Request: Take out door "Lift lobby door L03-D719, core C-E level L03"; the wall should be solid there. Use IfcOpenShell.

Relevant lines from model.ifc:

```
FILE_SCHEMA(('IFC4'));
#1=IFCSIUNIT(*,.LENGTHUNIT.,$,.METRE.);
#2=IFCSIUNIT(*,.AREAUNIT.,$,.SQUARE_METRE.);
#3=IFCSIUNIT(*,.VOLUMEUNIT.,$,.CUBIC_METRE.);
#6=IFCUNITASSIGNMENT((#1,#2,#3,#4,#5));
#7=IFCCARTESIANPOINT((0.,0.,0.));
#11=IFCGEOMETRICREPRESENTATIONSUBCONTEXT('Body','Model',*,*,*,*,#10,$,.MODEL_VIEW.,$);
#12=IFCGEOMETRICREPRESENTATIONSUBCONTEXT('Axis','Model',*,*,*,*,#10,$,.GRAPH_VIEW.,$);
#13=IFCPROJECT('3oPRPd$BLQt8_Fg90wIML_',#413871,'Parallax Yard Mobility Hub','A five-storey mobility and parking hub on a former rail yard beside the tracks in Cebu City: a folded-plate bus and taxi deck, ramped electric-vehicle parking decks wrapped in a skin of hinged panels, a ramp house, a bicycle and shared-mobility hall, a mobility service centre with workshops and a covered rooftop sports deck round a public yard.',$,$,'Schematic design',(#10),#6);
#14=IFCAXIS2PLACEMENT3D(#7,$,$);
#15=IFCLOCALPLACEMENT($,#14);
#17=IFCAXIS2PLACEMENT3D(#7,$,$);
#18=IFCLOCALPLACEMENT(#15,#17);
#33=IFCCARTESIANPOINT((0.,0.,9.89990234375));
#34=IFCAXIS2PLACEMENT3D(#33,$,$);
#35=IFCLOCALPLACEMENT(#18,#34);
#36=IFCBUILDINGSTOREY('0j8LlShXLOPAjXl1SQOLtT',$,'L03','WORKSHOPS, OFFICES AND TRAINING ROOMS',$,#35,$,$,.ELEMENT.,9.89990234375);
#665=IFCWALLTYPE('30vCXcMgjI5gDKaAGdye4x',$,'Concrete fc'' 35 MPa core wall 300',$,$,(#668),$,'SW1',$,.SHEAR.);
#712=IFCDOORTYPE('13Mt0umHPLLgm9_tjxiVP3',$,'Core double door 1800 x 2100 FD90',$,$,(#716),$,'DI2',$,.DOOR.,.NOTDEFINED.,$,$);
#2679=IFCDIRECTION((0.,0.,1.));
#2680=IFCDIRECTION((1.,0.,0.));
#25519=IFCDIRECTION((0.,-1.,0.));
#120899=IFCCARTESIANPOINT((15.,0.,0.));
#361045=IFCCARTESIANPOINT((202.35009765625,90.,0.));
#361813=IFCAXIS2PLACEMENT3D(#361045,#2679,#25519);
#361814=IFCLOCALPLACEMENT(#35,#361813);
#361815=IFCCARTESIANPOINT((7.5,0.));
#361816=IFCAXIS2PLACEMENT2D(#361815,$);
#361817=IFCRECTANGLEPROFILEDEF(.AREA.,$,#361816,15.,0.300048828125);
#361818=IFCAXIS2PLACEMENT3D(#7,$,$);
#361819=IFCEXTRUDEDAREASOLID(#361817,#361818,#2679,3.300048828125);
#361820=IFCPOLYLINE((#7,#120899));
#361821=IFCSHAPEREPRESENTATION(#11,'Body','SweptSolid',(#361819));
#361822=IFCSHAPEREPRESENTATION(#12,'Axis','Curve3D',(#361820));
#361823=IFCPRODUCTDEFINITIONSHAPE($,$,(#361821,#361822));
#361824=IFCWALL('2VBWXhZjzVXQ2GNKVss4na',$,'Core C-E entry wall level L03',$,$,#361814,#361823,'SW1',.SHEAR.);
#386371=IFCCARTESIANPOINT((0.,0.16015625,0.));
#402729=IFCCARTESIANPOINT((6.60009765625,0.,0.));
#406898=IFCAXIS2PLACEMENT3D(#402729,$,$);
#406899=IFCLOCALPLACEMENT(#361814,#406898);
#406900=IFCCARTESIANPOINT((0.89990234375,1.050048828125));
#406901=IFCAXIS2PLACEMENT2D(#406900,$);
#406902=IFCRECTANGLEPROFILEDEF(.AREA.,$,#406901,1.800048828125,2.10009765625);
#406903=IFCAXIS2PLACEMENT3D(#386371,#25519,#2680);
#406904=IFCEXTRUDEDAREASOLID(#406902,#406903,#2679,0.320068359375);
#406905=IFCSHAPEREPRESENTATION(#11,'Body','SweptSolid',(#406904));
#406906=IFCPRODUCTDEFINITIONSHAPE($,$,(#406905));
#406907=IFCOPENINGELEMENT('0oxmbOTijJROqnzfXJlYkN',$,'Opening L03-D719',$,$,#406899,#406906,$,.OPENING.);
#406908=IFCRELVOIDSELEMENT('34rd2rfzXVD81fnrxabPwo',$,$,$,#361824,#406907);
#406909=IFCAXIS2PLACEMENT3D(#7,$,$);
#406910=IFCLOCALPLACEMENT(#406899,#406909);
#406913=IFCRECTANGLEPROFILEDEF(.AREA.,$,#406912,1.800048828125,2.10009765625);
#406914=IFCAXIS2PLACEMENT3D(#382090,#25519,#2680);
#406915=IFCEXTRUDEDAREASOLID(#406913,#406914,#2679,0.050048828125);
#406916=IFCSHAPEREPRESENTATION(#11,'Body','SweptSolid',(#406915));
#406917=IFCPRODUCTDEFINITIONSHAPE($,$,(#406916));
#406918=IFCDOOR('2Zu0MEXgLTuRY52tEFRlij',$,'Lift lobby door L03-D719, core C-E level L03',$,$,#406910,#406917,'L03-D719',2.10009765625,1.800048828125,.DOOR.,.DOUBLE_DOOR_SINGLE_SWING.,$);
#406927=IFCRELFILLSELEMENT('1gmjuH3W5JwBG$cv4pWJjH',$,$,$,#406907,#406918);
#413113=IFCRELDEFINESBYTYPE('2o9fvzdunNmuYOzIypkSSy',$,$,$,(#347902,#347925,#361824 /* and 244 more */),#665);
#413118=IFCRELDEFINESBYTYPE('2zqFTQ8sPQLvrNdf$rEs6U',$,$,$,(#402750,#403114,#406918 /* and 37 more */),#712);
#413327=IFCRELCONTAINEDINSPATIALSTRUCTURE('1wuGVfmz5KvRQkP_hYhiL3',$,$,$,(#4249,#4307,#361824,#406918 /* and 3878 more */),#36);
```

```python
import ifcopenshell
import ifcopenshell.api.feature
import ifcopenshell.api.root
import ifcopenshell.geom
import ifcopenshell.util.shape

model = ifcopenshell.open("model.ifc")
settings = ifcopenshell.geom.settings()


def volume(element):
    """Net volume in cubic metres, openings subtracted."""
    shape = ifcopenshell.geom.create_shape(settings, element)
    return ifcopenshell.util.shape.get_volume(shape.geometry)


door = model.by_guid("2Zu0MEXgLTuRY52tEFRlij")
opening = door.FillsVoids[0].RelatingOpeningElement
wall = opening.VoidsElements[0].RelatingBuildingElement
before = volume(wall)

ifcopenshell.api.root.remove_product(model, product=door)
ifcopenshell.api.feature.remove_feature(model, feature=opening)

after = volume(wall)

print(f"wall volume {before:.3f} -> {after:.3f} m3")

model.write("model_updated.ifc")
```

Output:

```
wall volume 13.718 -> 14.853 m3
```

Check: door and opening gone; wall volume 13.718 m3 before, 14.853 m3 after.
